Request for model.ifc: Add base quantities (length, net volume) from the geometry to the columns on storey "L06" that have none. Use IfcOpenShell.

First a look at what the model holds.

```python
import ifcopenshell
import ifcopenshell.util.element
import ifcopenshell.util.unit

model = ifcopenshell.open("model.ifc")
print(model.schema)
for unit_type in ("LENGTHUNIT", "AREAUNIT", "VOLUMEUNIT"):
    print(unit_type, ifcopenshell.util.unit.calculate_unit_scale(model, unit_type))
storey = next(s for s in model.by_type("IfcBuildingStorey") if s.Name == "L06")
columns = [e for e in ifcopenshell.util.element.get_decomposition(storey) if e.is_a("IfcColumn")]
for e in sorted(columns, key=lambda e: e.id()):
    print(e.id(), e.is_a(), e.Name, list(ifcopenshell.util.element.get_psets(e, qtos_only=True)), sep=" | ")
```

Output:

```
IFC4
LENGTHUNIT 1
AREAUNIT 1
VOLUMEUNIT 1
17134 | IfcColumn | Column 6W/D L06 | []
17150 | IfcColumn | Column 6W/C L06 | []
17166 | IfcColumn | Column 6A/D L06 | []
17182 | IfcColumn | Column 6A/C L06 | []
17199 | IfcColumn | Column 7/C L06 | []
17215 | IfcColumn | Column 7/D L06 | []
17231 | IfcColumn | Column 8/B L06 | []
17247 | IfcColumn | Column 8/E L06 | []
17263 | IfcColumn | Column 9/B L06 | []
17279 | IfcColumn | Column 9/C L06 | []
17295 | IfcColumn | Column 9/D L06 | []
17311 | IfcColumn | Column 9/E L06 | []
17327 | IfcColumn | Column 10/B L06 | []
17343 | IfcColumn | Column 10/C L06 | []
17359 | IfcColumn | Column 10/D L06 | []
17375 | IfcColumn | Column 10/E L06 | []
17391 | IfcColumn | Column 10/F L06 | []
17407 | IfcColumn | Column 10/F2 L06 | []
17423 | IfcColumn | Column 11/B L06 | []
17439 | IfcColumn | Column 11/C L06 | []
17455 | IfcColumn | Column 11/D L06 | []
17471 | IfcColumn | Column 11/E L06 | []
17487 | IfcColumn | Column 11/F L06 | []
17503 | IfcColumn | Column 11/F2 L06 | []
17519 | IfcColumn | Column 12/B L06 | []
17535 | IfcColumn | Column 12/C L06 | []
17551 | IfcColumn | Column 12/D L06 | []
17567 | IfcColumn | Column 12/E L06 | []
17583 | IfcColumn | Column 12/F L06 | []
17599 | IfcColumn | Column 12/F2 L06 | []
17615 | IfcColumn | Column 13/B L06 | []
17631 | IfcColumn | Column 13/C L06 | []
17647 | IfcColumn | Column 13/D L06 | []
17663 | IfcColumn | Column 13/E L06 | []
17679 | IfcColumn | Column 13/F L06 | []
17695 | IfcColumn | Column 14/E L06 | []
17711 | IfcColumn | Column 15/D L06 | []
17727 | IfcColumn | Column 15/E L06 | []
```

```python
import ifcopenshell
import ifcopenshell.api.pset
import ifcopenshell.geom
import ifcopenshell.util.element
import ifcopenshell.util.shape
import ifcopenshell.util.unit

model = ifcopenshell.open("model.ifc")
unit_scale = ifcopenshell.util.unit.calculate_unit_scale(model)
volume_scale = ifcopenshell.util.unit.calculate_unit_scale(model, "VOLUMEUNIT")
settings = ifcopenshell.geom.settings()

storey = next(s for s in model.by_type("IfcBuildingStorey") if s.Name == "L06")
columns = [e for e in ifcopenshell.util.element.get_decomposition(storey) if e.is_a("IfcColumn")]

for e in sorted(columns, key=lambda e: e.id()):
    if ifcopenshell.util.element.get_psets(e, qtos_only=True, should_inherit=False):
        continue
    # Geometry comes back in metres, in the element's own axes.
    shape = ifcopenshell.geom.create_shape(settings, e)
    values = {
        "Length": ifcopenshell.util.shape.get_z(shape.geometry) / unit_scale,
        "NetVolume": ifcopenshell.util.shape.get_volume(shape.geometry) / volume_scale,
    }
    qto = ifcopenshell.api.pset.add_qto(model, product=e, name="Qto_ColumnBaseQuantities")
    ifcopenshell.api.pset.edit_qto(model, qto=qto, properties=values)
    print(e.id(), {k: round(v, 3) for k, v in values.items()})

model.write("model_rev.ifc")
```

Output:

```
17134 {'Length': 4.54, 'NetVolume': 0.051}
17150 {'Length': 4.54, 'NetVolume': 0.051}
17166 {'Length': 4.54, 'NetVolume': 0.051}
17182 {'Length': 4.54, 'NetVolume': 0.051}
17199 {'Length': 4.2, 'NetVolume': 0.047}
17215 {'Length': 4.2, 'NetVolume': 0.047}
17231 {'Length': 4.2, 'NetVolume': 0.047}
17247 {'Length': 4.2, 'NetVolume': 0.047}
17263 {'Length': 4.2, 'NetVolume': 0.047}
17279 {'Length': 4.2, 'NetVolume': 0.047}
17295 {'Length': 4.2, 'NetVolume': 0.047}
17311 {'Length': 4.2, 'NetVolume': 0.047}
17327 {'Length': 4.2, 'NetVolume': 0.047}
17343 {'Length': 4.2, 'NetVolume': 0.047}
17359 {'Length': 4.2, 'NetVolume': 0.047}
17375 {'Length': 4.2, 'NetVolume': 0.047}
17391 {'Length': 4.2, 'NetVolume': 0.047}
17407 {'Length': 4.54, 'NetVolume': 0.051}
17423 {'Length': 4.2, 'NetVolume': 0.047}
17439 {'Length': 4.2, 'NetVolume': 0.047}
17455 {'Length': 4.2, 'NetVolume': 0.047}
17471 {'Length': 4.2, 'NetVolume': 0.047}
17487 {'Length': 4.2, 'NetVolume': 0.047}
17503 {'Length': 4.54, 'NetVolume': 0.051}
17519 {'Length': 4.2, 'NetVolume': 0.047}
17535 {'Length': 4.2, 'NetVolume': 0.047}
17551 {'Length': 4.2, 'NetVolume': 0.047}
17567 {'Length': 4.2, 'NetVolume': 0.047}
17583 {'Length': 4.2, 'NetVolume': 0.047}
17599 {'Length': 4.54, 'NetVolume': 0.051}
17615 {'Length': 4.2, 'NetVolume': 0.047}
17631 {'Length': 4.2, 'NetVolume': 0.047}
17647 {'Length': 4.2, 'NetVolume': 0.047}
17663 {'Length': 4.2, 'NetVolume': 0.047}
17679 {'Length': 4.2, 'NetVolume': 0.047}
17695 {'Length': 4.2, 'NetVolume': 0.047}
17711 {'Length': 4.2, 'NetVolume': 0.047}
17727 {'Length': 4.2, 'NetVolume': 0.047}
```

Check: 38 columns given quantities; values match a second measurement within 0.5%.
